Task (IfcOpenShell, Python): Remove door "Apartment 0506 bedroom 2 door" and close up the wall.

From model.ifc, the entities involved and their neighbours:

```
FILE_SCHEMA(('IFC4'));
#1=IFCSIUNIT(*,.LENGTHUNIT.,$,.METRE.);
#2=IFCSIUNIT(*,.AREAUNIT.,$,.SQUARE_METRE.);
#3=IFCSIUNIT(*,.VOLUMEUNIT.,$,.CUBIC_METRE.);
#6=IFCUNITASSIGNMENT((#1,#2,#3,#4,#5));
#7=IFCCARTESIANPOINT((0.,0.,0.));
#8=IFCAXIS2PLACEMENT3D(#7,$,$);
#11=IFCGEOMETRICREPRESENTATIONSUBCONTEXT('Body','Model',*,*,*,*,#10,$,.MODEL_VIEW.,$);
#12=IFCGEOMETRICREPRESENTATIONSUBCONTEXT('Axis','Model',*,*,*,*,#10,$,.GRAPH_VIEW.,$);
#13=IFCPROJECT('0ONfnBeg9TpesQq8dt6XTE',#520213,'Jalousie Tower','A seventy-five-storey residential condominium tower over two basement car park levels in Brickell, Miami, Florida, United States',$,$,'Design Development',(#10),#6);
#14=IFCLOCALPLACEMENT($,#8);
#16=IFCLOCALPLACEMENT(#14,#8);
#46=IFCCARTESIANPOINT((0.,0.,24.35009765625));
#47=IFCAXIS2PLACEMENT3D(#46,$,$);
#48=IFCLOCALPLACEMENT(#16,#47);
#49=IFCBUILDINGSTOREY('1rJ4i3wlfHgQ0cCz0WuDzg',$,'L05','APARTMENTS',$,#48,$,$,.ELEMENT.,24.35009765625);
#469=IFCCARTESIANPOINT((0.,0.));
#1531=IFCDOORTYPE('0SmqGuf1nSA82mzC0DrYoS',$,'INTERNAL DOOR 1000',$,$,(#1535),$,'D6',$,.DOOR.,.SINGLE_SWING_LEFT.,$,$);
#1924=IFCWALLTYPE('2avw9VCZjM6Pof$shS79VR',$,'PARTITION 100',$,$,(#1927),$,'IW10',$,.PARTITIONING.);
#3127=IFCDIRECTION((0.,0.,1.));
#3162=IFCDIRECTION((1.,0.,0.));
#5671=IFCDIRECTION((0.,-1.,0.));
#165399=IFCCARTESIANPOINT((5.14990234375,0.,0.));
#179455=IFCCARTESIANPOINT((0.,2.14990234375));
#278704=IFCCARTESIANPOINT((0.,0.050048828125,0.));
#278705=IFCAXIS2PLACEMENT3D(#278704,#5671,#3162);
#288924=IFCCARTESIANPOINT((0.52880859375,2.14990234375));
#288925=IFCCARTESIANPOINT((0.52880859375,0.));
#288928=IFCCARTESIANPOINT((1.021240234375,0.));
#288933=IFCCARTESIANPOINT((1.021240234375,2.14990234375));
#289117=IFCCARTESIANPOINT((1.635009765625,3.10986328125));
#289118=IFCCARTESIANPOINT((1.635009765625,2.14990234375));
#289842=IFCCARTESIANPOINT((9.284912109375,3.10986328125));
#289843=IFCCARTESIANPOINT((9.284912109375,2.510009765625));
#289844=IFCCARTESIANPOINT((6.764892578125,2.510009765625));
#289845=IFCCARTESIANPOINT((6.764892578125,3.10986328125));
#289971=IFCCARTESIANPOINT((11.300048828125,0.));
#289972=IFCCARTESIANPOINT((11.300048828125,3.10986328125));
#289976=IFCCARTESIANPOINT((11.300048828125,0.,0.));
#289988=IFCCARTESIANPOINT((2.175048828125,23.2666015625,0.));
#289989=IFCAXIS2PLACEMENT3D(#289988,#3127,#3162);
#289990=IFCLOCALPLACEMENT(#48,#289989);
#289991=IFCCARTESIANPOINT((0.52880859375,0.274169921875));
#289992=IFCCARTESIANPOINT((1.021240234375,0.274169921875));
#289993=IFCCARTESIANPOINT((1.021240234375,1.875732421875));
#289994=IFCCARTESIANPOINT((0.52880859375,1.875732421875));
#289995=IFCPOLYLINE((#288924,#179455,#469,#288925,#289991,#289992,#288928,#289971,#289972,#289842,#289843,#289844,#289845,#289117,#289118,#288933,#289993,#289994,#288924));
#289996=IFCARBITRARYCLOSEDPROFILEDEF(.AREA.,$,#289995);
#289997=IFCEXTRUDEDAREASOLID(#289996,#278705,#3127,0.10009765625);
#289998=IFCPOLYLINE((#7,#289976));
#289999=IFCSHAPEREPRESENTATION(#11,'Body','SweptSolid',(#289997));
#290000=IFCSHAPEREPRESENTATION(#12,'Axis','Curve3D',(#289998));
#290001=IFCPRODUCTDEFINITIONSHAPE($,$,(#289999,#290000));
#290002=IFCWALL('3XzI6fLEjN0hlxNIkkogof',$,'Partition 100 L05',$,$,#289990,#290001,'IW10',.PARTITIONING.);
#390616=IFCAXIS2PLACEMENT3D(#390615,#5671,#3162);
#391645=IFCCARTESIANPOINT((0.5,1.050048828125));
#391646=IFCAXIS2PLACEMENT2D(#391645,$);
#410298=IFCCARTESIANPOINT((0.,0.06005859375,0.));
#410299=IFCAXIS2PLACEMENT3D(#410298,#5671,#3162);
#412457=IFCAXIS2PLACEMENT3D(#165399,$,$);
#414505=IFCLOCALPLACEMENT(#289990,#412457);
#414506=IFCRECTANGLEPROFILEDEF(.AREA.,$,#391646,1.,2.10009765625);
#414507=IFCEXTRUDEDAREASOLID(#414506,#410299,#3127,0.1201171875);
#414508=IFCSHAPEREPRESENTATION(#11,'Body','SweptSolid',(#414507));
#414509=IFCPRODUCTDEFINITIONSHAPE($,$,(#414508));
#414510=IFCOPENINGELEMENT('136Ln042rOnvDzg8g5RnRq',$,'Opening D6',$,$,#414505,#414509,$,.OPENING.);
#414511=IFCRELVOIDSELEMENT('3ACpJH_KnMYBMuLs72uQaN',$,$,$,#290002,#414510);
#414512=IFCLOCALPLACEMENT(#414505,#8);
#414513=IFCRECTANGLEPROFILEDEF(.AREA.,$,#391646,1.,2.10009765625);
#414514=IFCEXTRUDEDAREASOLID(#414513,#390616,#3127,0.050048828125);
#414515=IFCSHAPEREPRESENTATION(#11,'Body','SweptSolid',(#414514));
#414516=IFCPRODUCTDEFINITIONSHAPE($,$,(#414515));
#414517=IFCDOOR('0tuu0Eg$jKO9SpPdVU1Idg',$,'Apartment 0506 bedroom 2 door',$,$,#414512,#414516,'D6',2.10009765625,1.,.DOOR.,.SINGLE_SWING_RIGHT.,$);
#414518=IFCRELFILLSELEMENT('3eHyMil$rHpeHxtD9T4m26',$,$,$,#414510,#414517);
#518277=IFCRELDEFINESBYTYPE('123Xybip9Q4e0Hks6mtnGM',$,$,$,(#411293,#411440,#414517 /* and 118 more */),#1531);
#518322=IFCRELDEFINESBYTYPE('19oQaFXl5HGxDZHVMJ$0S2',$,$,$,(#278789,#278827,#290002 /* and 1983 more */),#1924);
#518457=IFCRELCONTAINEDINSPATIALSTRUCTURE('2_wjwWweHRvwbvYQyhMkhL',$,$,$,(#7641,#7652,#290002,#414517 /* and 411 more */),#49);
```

```python
import ifcopenshell
import ifcopenshell.api.feature
import ifcopenshell.api.root
import ifcopenshell.geom
import ifcopenshell.util.shape

model = ifcopenshell.open("model.ifc")
settings = ifcopenshell.geom.settings()


def volume(element):
    """Net volume in cubic metres, openings subtracted."""
    shape = ifcopenshell.geom.create_shape(settings, element)
    return ifcopenshell.util.shape.get_volume(shape.geometry)


door = model.by_id(414517)
opening = door.FillsVoids[0].RelatingOpeningElement
wall = opening.VoidsElements[0].RelatingBuildingElement
before = volume(wall)

ifcopenshell.api.root.remove_product(model, product=door)
ifcopenshell.api.feature.remove_feature(model, feature=opening)

after = volume(wall)

print(f"wall volume {before:.3f} -> {after:.3f} m3")

model.write("model_updated.ifc")
```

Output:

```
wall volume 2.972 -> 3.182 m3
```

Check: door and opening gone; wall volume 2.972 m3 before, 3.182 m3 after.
